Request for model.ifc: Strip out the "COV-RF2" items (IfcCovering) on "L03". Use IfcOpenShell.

First a look at what the model holds.

```python
import ifcopenshell
import ifcopenshell.util.element

model = ifcopenshell.open("model.ifc")
print(model.schema)
storey = next(s for s in model.by_type("IfcBuildingStorey") if s.Name == "L03")
coverings = [e for e in ifcopenshell.util.element.get_decomposition(storey) if e.is_a("IfcCovering")]
seen = {}
for e in coverings:
    element_type = ifcopenshell.util.element.get_type(e)
    name = element_type.Name if element_type not in (None, e) else None
    seen[name] = seen.get(name, 0) + 1
for name, count in sorted(seen.items(), key=str):
    print(count, "x", name)
```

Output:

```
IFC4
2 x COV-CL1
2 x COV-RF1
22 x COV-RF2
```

```python
import ifcopenshell
import ifcopenshell.api.root
import ifcopenshell.util.element

model = ifcopenshell.open("model.ifc")

storey = next(s for s in model.by_type("IfcBuildingStorey") if s.Name == "L03")
coverings = [e for e in ifcopenshell.util.element.get_decomposition(storey) if e.is_a("IfcCovering")]
targets = [e for e in coverings if (t := ifcopenshell.util.element.get_type(e)) not in (None, e) and t.Name == "COV-RF2"]

for e in targets:
    ifcopenshell.api.root.remove_product(model, product=e)
print(len(targets), "removed")

model.write("model_rev.ifc")
```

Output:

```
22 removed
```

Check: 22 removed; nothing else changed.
